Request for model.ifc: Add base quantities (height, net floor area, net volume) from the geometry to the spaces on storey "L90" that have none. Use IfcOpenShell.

First a look at what the model holds.

```python
import ifcopenshell
import ifcopenshell.util.element
import ifcopenshell.util.unit

model = ifcopenshell.open("model.ifc")
print(model.schema)
for unit_type in ("LENGTHUNIT", "AREAUNIT", "VOLUMEUNIT"):
    print(unit_type, ifcopenshell.util.unit.calculate_unit_scale(model, unit_type))
storey = next(s for s in model.by_type("IfcBuildingStorey") if s.Name == "L90")
spaces = [e for e in ifcopenshell.util.element.get_decomposition(storey) if e.is_a("IfcSpace")]
for e in sorted(spaces, key=lambda e: e.id()):
    print(e.id(), e.is_a(), e.Name, list(ifcopenshell.util.element.get_psets(e, qtos_only=True)), sep=" | ")
```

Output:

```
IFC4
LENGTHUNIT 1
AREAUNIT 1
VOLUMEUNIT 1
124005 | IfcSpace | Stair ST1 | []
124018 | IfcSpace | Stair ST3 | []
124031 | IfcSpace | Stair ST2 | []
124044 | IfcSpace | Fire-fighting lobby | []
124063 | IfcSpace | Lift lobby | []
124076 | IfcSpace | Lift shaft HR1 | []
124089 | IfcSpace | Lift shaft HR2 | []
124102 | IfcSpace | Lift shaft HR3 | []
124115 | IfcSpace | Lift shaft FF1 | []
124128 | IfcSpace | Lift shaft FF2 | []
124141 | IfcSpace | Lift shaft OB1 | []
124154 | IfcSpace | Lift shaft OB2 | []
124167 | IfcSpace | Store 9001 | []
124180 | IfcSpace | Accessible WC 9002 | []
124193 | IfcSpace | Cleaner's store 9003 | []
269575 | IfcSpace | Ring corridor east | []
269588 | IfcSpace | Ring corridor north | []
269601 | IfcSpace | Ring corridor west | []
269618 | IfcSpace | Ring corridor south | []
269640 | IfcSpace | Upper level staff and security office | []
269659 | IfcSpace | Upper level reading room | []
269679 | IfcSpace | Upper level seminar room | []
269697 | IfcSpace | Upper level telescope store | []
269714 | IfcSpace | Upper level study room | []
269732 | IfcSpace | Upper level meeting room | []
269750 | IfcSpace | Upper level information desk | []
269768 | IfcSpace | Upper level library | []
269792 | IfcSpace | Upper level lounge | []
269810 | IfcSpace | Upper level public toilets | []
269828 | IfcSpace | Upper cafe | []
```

```python
import ifcopenshell
import ifcopenshell.api.pset
import ifcopenshell.geom
import ifcopenshell.util.element
import ifcopenshell.util.shape
import ifcopenshell.util.unit

model = ifcopenshell.open("model.ifc")
unit_scale = ifcopenshell.util.unit.calculate_unit_scale(model)
area_scale = ifcopenshell.util.unit.calculate_unit_scale(model, "AREAUNIT")
volume_scale = ifcopenshell.util.unit.calculate_unit_scale(model, "VOLUMEUNIT")
settings = ifcopenshell.geom.settings()

storey = next(s for s in model.by_type("IfcBuildingStorey") if s.Name == "L90")
spaces = [e for e in ifcopenshell.util.element.get_decomposition(storey) if e.is_a("IfcSpace")]

for e in sorted(spaces, key=lambda e: e.id()):
    if ifcopenshell.util.element.get_psets(e, qtos_only=True, should_inherit=False):
        continue
    # Geometry comes back in metres, in the element's own axes.
    shape = ifcopenshell.geom.create_shape(settings, e)
    values = {
        "Height": ifcopenshell.util.shape.get_z(shape.geometry) / unit_scale,
        "NetFloorArea": ifcopenshell.util.shape.get_footprint_area(shape.geometry) / area_scale,
        "NetVolume": ifcopenshell.util.shape.get_volume(shape.geometry) / volume_scale,
    }
    qto = ifcopenshell.api.pset.add_qto(model, product=e, name="Qto_SpaceBaseQuantities")
    ifcopenshell.api.pset.edit_qto(model, qto=qto, properties=values)
    print(e.id(), {k: round(v, 3) for k, v in values.items()})

model.write("model_updated.ifc")
```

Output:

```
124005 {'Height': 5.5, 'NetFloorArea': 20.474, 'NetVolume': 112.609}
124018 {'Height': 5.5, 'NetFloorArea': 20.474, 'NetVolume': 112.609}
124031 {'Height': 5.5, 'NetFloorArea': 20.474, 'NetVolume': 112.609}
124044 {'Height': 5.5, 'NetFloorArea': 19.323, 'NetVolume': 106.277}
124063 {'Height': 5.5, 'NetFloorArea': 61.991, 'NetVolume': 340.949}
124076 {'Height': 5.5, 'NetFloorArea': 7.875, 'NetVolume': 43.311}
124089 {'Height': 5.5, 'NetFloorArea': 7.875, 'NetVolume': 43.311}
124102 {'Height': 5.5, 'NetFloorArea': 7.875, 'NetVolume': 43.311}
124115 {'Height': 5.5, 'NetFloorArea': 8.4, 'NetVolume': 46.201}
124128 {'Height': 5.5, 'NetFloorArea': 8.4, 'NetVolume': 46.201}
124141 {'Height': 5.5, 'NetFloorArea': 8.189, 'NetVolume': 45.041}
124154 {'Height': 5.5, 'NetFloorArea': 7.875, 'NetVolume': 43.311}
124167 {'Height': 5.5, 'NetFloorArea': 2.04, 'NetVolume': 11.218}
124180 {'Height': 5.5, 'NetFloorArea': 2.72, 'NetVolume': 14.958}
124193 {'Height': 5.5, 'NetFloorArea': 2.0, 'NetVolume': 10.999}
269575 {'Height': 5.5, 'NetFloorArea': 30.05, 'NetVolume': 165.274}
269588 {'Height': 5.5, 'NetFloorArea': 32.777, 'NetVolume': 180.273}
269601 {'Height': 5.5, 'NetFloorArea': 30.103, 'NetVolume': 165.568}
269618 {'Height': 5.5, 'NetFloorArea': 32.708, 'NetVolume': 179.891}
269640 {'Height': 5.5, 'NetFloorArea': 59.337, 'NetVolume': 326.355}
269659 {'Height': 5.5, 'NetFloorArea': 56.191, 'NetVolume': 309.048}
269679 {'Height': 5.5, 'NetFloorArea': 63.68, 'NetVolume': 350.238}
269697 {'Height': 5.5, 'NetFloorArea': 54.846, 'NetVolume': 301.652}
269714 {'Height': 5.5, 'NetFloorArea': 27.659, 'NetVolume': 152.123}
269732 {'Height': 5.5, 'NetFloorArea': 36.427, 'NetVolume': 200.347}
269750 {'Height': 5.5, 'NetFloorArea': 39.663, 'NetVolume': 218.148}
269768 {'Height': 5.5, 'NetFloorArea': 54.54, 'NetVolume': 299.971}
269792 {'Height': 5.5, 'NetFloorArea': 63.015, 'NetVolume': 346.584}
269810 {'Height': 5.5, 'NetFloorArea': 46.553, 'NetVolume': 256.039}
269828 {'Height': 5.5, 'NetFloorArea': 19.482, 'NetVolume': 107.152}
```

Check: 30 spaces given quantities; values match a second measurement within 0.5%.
